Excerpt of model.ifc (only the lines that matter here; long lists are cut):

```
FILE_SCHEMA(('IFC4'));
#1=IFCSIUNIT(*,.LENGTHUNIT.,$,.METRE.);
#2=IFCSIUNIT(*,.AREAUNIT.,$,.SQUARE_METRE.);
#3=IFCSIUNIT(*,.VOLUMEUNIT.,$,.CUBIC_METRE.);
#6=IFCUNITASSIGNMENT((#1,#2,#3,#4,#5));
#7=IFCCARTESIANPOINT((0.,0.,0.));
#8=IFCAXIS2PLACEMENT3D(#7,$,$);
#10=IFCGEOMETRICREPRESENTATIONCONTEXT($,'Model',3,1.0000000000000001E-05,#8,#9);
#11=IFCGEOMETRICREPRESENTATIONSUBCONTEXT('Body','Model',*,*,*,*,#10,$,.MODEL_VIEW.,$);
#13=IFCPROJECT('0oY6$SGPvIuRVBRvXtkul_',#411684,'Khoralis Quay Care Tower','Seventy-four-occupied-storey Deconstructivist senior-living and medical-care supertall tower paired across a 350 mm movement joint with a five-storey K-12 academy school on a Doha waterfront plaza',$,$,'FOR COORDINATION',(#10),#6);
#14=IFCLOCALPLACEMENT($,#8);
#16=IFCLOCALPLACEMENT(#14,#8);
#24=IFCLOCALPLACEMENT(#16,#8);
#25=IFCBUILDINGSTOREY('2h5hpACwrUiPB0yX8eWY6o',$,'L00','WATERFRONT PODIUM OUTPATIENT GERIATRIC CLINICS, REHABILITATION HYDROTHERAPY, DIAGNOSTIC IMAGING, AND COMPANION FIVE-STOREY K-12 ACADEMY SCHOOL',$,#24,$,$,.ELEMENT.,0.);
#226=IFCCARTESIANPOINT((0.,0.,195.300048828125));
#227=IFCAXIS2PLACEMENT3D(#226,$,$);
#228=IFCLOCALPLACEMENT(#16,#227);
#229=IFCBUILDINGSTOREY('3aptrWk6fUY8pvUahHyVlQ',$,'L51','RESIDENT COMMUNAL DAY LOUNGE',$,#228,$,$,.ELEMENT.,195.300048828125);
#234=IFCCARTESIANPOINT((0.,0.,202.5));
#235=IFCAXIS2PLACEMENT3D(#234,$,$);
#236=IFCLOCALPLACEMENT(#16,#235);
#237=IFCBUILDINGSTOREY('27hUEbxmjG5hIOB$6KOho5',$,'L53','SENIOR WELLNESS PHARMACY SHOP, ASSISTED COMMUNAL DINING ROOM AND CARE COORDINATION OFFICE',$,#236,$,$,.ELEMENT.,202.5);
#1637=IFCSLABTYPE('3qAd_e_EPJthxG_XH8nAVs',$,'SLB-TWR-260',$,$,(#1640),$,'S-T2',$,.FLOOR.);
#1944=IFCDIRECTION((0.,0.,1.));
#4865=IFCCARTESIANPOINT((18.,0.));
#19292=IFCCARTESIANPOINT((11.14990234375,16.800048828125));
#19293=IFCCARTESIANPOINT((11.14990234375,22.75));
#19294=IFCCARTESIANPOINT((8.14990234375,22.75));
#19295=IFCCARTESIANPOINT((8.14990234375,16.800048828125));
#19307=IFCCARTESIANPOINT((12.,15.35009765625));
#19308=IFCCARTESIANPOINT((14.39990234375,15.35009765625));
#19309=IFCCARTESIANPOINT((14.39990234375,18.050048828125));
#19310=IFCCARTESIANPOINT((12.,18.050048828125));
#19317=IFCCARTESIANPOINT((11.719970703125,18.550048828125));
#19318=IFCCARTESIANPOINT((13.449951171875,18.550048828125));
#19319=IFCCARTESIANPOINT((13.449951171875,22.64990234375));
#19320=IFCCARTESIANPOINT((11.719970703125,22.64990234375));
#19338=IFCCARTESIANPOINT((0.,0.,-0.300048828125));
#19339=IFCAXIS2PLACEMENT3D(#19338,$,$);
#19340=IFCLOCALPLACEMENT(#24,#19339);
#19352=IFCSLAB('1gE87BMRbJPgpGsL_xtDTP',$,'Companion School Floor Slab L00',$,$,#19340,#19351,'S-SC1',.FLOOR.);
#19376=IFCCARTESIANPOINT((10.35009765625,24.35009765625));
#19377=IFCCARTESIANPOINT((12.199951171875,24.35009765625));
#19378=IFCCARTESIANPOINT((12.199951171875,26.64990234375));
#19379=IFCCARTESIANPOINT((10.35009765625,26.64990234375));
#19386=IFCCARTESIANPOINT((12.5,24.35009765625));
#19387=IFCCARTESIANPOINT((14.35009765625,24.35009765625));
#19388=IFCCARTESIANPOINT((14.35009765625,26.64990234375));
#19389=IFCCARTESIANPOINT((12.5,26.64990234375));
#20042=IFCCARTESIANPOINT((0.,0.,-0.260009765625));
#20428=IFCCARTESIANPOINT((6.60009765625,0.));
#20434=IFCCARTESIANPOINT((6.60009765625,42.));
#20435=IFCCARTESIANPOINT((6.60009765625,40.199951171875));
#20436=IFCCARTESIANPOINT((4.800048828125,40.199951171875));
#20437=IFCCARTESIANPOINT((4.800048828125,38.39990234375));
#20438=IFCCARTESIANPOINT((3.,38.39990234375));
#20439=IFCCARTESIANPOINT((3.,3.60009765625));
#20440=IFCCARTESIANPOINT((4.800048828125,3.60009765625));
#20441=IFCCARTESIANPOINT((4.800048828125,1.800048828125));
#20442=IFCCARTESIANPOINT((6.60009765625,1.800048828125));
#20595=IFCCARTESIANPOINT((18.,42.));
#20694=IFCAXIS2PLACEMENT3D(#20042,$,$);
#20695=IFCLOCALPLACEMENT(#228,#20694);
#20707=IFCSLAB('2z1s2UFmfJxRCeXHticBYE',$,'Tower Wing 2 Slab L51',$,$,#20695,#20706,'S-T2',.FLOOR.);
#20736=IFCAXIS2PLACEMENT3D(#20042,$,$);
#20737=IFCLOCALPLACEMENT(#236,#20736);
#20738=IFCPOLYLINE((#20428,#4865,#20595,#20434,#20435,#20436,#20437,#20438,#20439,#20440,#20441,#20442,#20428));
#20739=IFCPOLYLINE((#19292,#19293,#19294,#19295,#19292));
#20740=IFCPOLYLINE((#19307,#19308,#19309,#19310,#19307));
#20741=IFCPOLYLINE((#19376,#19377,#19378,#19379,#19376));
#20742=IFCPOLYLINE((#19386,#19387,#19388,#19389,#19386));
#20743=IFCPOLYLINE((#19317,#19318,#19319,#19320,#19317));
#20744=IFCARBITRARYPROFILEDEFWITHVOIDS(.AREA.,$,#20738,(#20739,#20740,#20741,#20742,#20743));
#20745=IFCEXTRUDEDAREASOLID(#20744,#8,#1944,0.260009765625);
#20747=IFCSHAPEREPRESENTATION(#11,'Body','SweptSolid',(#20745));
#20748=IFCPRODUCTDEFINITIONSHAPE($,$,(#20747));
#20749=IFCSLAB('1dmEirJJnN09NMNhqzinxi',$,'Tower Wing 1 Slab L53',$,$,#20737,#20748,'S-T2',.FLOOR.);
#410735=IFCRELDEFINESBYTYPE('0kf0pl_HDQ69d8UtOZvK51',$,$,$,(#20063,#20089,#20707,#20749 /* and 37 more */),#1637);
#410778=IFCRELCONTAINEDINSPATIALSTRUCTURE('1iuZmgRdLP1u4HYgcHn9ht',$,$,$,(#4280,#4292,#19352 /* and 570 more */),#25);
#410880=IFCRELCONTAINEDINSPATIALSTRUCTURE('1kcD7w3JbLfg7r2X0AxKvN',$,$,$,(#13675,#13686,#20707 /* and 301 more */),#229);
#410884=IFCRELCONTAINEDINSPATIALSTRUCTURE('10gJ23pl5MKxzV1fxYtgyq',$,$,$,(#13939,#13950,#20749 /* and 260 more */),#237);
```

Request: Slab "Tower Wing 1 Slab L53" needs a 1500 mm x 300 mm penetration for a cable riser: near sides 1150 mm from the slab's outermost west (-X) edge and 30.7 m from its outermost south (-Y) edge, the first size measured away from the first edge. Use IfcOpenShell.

```python
import numpy as np
import ifcopenshell
import ifcopenshell.api.feature
import ifcopenshell.api.geometry
import ifcopenshell.api.root
import ifcopenshell.geom
import ifcopenshell.util.placement
import ifcopenshell.util.representation
import ifcopenshell.util.shape
import ifcopenshell.util.unit

model = ifcopenshell.open("model.ifc")
unit_scale = ifcopenshell.util.unit.calculate_unit_scale(model)
settings = ifcopenshell.geom.settings()


def volume(element):
    """Net volume in cubic metres, openings subtracted."""
    shape = ifcopenshell.geom.create_shape(settings, element)
    return ifcopenshell.util.shape.get_volume(shape.geometry)


slab = model.by_guid("1dmEirJJnN09NMNhqzinxi")
before = volume(slab)

# Extent in the slab's own axes, in metres. The edges named are its -X and -Y sides.
slab_shape = ifcopenshell.geom.create_shape(settings, slab)
vertices = ifcopenshell.util.shape.get_vertices(slab_shape.geometry)
x_min, y_min, bottom = vertices.min(axis=0)
top = vertices[:, 2].max()

opening = ifcopenshell.api.root.create_entity(model, ifc_class="IfcOpeningElement", name="Cable riser opening", predefined_type="OPENING")
context = ifcopenshell.util.representation.get_context(model, "Model", "Body", "MODEL_VIEW")
width, depth = 1.5, 0.3
outline = [(0.0, 0.0), (width, 0.0), (width, depth), (0.0, depth), (0.0, 0.0)]
# Overshoot both faces by 50 mm so the cut is clean.
shape = ifcopenshell.api.geometry.add_slab_representation(
    model, context=context, depth=top - bottom + 0.1, polyline=outline
)
ifcopenshell.api.geometry.assign_representation(model, product=opening, representation=shape)

matrix = ifcopenshell.util.placement.get_local_placement(slab.ObjectPlacement)
matrix[:, 3] = matrix @ np.append(np.array([x_min + 1.15, y_min + 30.7, bottom - 0.05]) / unit_scale, 1.0)
ifcopenshell.api.geometry.edit_object_placement(model, product=opening, matrix=matrix, is_si=False)
ifcopenshell.api.feature.add_feature(model, feature=opening, element=slab)

after = volume(slab)

print(f"slab volume {before:.3f} -> {after:.3f} m3")

model.write("model_v2.ifc")
```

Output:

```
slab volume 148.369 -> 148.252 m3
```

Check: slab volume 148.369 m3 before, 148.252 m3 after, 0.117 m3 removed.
